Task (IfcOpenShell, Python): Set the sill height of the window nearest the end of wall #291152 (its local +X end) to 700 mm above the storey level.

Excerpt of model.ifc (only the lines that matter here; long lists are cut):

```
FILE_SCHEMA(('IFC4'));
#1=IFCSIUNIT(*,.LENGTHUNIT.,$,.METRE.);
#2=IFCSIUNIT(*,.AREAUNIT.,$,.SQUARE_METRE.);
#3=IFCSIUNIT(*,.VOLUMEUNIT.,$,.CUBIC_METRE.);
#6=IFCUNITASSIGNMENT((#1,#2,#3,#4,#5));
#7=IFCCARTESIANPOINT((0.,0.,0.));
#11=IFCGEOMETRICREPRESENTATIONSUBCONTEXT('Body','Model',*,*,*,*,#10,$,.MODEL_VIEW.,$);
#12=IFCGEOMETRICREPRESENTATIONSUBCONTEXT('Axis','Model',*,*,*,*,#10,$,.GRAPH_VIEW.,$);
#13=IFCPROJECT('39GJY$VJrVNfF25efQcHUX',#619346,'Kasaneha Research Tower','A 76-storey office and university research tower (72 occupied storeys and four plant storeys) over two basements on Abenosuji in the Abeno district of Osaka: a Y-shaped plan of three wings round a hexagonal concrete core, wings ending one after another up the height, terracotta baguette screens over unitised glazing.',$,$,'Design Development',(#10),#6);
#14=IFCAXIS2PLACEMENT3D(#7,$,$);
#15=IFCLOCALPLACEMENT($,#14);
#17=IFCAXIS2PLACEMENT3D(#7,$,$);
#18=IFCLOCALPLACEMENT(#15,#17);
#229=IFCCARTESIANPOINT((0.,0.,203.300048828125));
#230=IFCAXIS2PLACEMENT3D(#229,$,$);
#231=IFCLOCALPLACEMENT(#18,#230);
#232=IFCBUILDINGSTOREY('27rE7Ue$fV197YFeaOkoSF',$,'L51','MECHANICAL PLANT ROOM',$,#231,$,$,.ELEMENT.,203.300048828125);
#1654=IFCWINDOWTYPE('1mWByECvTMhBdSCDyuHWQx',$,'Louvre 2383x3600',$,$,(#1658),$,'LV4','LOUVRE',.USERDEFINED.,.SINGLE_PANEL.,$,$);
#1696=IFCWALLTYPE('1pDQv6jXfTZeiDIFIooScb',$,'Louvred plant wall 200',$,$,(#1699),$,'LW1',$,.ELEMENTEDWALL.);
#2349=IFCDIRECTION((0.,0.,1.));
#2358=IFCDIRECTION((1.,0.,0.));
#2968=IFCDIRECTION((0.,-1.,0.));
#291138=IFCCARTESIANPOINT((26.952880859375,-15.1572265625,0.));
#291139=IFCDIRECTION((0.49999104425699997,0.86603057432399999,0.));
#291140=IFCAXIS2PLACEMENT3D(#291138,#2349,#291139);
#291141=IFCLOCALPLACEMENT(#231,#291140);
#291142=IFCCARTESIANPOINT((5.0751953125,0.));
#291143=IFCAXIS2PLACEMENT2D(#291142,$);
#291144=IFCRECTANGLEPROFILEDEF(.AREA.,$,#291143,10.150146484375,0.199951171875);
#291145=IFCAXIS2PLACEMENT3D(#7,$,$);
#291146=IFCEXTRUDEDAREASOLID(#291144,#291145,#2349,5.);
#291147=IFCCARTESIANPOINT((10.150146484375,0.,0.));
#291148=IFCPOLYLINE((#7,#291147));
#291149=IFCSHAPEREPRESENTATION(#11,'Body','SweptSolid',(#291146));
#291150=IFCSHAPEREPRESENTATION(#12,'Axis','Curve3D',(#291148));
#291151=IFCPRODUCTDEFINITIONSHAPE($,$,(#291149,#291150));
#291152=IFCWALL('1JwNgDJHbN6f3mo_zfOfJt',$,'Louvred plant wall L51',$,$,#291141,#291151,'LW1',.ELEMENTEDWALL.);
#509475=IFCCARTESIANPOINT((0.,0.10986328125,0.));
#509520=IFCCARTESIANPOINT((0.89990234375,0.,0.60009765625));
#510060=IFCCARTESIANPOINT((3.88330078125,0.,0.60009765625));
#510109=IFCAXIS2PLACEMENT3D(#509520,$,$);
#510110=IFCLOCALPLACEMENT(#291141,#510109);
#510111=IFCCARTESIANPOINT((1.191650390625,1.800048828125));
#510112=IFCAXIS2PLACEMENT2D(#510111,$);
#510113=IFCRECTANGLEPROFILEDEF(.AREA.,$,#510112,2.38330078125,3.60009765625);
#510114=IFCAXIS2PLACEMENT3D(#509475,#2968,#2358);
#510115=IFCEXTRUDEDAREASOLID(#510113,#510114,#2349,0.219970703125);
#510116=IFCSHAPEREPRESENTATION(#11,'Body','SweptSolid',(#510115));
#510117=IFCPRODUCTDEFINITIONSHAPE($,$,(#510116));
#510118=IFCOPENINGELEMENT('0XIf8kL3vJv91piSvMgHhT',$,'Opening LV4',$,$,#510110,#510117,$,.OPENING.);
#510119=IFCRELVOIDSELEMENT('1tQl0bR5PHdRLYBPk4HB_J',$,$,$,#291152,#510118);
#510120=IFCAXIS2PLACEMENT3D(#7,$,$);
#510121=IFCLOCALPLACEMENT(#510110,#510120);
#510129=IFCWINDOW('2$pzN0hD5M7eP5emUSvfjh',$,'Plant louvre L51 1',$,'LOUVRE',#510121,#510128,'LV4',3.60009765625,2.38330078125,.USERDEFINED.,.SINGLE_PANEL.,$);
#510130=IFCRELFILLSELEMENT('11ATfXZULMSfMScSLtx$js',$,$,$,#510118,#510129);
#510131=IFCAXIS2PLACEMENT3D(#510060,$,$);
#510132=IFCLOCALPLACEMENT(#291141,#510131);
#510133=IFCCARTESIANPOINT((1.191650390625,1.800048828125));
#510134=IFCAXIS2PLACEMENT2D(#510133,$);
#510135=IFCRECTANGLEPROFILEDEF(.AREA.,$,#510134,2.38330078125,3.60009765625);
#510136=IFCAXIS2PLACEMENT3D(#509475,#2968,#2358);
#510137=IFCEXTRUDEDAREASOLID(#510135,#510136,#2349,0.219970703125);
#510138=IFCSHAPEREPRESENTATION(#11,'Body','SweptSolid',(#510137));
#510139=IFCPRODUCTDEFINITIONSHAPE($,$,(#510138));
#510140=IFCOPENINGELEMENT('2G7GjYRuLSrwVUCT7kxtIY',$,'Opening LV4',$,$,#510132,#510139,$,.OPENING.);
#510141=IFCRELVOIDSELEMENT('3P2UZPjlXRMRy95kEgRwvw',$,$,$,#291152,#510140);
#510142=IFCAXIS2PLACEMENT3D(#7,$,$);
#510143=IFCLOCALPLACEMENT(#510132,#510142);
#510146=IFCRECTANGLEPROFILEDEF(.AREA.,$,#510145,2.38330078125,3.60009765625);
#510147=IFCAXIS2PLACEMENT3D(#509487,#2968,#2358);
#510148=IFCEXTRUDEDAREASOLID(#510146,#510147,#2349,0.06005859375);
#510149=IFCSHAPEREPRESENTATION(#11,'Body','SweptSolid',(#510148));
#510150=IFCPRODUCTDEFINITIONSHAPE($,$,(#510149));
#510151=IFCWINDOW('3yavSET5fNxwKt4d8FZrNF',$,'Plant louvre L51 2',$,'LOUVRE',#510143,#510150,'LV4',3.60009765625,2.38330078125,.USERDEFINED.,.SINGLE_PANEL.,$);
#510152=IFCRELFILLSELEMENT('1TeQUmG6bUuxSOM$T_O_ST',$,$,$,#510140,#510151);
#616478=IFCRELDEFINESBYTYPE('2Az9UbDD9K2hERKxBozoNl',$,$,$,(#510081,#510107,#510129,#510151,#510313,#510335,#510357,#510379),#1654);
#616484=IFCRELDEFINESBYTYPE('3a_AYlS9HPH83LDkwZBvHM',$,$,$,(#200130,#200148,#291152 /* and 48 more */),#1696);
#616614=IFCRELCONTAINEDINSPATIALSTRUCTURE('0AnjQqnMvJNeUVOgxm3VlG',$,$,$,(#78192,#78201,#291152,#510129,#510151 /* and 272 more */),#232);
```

```python
import numpy as np
import ifcopenshell
import ifcopenshell.api.geometry
import ifcopenshell.geom
import ifcopenshell.util.element
import ifcopenshell.util.placement
import ifcopenshell.util.shape
import ifcopenshell.util.unit

model = ifcopenshell.open("model.ifc")
unit_scale = ifcopenshell.util.unit.calculate_unit_scale(model)

window = model.by_guid("3yavSET5fNxwKt4d8FZrNF")
opening = window.FillsVoids[0].RelatingOpeningElement
storey = ifcopenshell.util.element.get_container(window, ifc_class="IfcBuildingStorey")
level = ifcopenshell.util.placement.get_local_placement(storey.ObjectPlacement)[2, 3]

# The opening's origin need not be at the sill, so measure its lowest point.
shape = ifcopenshell.geom.create_shape(ifcopenshell.geom.settings(), opening)
bottom = ifcopenshell.util.shape.get_shape_bottom_elevation(shape, shape.geometry) / unit_scale
dz = level + 0.7 / unit_scale - bottom

shift = np.array([0.0, 0.0, dz])
# The window is placed relative to its opening, so it follows when the opening moves.
matrix = ifcopenshell.util.placement.get_local_placement(opening.ObjectPlacement)
matrix[:3, 3] += shift
ifcopenshell.api.geometry.edit_object_placement(
    model, product=opening, matrix=matrix, is_si=False, should_transform_children=True
)

print(f"moved by {dz * unit_scale:+.3f} m")

model.write("model_updated.ifc")
```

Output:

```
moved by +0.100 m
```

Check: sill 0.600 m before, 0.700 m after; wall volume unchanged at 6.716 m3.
